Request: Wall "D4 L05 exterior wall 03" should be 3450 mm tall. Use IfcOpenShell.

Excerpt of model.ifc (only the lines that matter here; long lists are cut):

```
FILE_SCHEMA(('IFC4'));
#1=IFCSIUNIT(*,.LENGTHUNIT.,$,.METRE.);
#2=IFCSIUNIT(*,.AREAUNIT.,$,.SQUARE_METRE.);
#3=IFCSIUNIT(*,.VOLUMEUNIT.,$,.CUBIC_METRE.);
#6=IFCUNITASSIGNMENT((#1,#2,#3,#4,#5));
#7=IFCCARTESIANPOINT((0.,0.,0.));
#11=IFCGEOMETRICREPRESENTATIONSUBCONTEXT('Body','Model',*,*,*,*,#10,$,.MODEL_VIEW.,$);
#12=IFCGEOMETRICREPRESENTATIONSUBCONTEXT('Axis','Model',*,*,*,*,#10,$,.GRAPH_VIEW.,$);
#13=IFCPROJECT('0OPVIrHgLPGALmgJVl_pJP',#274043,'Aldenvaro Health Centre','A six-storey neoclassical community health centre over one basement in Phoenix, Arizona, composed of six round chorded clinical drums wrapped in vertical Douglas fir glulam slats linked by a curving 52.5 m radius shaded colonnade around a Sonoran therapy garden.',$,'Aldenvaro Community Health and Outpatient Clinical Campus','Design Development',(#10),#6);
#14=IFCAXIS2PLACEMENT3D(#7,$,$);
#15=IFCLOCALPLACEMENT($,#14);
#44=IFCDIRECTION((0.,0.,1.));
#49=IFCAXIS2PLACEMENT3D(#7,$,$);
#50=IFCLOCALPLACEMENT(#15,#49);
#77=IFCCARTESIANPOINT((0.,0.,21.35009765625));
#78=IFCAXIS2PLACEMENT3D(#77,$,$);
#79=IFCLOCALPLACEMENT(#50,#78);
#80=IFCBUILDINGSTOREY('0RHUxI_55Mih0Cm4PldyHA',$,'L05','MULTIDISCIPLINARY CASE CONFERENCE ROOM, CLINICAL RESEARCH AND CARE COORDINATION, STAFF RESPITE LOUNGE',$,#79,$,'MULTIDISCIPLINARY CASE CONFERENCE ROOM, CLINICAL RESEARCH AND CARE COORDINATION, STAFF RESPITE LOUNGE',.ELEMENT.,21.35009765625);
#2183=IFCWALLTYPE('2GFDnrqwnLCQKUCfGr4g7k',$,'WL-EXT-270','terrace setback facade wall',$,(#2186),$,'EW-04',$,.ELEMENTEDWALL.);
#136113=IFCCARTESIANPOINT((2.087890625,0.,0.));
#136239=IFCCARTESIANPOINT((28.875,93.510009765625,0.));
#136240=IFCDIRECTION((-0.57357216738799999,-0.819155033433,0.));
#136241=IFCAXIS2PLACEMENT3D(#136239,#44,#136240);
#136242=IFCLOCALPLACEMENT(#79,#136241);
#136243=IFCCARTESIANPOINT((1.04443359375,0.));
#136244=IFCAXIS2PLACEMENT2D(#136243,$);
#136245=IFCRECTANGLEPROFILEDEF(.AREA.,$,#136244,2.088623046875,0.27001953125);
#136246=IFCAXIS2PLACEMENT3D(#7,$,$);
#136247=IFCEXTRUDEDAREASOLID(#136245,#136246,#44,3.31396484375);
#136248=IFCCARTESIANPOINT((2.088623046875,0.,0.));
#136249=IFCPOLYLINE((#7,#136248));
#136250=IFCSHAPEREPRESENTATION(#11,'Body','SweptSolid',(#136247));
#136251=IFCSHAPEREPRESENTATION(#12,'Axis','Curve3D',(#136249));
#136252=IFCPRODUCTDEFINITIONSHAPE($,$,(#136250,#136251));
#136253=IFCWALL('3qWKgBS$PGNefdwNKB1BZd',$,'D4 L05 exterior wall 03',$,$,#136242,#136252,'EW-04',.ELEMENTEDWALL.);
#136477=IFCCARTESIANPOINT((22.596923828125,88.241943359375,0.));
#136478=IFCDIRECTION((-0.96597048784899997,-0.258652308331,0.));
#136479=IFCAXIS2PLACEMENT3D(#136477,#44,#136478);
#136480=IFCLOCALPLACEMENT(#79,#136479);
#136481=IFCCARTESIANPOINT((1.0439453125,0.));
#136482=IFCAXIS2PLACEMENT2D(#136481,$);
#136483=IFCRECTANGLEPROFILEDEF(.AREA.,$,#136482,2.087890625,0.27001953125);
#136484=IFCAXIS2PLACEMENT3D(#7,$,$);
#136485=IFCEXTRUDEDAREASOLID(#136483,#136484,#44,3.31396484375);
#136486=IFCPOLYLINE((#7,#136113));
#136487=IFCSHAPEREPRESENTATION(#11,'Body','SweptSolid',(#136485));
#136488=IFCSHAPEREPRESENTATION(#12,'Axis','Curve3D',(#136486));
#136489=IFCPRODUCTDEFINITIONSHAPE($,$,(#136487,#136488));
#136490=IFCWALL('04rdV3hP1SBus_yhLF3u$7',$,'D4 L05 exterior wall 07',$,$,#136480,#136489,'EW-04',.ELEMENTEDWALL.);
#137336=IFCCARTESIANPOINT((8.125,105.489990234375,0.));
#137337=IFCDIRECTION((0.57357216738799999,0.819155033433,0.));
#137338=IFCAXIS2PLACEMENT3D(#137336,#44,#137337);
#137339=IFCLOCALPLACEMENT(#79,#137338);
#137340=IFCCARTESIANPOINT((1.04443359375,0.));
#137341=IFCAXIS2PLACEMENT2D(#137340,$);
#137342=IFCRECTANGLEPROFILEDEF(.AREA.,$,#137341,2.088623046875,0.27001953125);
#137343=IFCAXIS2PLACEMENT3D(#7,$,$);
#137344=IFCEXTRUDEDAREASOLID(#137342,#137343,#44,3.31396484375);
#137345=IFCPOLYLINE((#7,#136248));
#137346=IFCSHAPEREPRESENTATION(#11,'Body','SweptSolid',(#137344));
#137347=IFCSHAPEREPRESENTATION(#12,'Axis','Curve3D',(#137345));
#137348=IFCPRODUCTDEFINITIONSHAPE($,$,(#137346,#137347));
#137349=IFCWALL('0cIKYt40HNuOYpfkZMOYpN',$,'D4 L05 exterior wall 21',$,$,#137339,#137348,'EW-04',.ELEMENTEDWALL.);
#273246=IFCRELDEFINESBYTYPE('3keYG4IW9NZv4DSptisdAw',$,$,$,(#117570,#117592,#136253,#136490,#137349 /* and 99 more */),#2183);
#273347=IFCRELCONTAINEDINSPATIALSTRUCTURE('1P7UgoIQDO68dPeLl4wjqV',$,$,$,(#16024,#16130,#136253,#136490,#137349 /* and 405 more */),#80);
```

```python
import ifcopenshell
import ifcopenshell.geom
import ifcopenshell.util.representation
import ifcopenshell.util.shape

model = ifcopenshell.open("model.ifc")
settings = ifcopenshell.geom.settings()


def volume(element):
    """Net volume in cubic metres, openings subtracted."""
    shape = ifcopenshell.geom.create_shape(settings, element)
    return ifcopenshell.util.shape.get_volume(shape.geometry)


wall = model.by_guid("3qWKgBS$PGNefdwNKB1BZd")
before = volume(wall)

body = ifcopenshell.util.representation.get_representation(wall, "Model", "Body")
solid = body.Items[0]
old_height = solid.Depth
solid.Depth = 3.45
after = volume(wall)

print(f"height {old_height:g} -> {solid.Depth:g}, volume {before:.3f} -> {after:.3f} m3")

model.write("model_rev.ifc")
```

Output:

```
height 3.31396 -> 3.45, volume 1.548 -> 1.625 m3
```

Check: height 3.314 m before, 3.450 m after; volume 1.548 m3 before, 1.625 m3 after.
